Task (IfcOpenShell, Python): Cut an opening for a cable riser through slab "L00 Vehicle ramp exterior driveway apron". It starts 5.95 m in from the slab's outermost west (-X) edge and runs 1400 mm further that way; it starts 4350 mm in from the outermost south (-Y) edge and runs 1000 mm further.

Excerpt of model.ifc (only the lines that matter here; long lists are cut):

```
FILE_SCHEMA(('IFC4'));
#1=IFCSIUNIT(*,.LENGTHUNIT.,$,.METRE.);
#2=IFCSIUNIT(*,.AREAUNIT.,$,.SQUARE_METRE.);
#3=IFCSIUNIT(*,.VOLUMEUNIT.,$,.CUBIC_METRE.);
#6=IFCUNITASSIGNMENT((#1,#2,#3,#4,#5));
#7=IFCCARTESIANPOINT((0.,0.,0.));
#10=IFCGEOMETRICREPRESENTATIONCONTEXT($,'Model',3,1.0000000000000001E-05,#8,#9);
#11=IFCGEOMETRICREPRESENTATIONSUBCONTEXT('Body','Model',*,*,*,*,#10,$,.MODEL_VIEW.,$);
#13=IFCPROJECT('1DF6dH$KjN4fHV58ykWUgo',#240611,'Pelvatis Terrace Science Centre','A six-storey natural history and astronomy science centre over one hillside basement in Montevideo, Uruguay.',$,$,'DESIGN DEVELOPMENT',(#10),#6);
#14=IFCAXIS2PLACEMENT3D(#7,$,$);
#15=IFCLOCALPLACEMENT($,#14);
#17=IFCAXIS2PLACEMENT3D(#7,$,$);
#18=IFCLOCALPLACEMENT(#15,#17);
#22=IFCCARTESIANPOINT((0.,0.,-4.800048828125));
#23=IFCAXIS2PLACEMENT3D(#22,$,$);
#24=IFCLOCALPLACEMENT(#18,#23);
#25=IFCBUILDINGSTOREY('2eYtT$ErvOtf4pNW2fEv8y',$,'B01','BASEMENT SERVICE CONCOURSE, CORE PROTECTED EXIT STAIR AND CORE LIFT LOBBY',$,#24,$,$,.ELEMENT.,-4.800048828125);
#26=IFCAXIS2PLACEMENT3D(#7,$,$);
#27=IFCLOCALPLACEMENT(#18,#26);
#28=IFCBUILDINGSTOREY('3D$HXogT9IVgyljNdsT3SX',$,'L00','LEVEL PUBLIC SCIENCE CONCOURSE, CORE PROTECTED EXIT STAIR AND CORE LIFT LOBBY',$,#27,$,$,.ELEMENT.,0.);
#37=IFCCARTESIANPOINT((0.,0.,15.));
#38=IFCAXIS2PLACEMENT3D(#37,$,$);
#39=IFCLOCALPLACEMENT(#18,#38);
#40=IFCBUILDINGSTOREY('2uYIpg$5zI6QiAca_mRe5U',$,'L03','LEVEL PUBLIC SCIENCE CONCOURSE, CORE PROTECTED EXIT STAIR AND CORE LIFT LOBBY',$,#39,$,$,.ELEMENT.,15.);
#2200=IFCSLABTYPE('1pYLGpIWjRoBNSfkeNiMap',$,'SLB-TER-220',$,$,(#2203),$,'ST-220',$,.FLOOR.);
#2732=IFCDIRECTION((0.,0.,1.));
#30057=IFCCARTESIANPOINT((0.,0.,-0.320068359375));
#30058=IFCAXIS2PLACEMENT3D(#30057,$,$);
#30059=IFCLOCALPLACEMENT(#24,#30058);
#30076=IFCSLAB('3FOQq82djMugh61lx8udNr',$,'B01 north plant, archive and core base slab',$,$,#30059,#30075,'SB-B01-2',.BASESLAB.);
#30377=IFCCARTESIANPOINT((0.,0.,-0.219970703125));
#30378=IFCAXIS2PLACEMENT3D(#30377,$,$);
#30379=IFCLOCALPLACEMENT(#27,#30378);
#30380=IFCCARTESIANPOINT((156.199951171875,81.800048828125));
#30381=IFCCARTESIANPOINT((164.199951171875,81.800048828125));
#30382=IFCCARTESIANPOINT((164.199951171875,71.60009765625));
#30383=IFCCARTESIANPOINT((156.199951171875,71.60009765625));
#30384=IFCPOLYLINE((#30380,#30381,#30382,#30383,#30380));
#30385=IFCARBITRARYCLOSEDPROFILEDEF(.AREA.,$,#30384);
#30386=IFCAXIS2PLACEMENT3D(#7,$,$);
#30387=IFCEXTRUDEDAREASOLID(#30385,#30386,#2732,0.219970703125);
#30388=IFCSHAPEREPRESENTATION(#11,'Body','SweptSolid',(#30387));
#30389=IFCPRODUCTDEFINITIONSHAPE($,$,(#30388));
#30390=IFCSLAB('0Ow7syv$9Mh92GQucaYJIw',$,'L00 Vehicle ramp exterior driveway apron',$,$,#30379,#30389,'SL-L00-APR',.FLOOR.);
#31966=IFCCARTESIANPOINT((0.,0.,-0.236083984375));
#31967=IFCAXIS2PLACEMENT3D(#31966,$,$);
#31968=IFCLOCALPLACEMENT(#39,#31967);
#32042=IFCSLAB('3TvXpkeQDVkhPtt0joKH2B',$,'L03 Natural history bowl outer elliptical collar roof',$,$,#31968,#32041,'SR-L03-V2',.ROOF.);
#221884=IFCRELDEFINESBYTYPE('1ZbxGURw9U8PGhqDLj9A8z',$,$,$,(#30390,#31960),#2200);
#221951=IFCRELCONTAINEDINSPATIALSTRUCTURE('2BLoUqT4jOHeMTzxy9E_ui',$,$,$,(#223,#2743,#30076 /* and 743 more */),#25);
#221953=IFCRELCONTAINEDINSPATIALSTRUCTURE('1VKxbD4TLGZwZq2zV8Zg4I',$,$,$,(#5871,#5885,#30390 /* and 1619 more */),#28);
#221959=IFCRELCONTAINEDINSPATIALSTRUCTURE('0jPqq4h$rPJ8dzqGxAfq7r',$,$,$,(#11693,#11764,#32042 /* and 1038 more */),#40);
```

```python
import numpy as np
import ifcopenshell
import ifcopenshell.api.feature
import ifcopenshell.api.geometry
import ifcopenshell.api.root
import ifcopenshell.geom
import ifcopenshell.util.placement
import ifcopenshell.util.representation
import ifcopenshell.util.shape
import ifcopenshell.util.unit

model = ifcopenshell.open("model.ifc")
unit_scale = ifcopenshell.util.unit.calculate_unit_scale(model)
settings = ifcopenshell.geom.settings()


def volume(element):
    """Net volume in cubic metres, openings subtracted."""
    shape = ifcopenshell.geom.create_shape(settings, element)
    return ifcopenshell.util.shape.get_volume(shape.geometry)


slab = model.by_guid("0Ow7syv$9Mh92GQucaYJIw")
before = volume(slab)

# Extent in the slab's own axes, in metres. The edges named are its -X and -Y sides.
slab_shape = ifcopenshell.geom.create_shape(settings, slab)
vertices = ifcopenshell.util.shape.get_vertices(slab_shape.geometry)
x_min, y_min, bottom = vertices.min(axis=0)
top = vertices[:, 2].max()

opening = ifcopenshell.api.root.create_entity(model, ifc_class="IfcOpeningElement", name="Cable riser opening", predefined_type="OPENING")
context = ifcopenshell.util.representation.get_context(model, "Model", "Body", "MODEL_VIEW")
width, depth = 1.4, 1
outline = [(0.0, 0.0), (width, 0.0), (width, depth), (0.0, depth), (0.0, 0.0)]
# Overshoot both faces by 50 mm so the cut is clean.
shape = ifcopenshell.api.geometry.add_slab_representation(
    model, context=context, depth=top - bottom + 0.1, polyline=outline
)
ifcopenshell.api.geometry.assign_representation(model, product=opening, representation=shape)

matrix = ifcopenshell.util.placement.get_local_placement(slab.ObjectPlacement)
matrix[:, 3] = matrix @ np.append(np.array([x_min + 5.95, y_min + 4.35, bottom - 0.05]) / unit_scale, 1.0)
ifcopenshell.api.geometry.edit_object_placement(model, product=opening, matrix=matrix, is_si=False)
ifcopenshell.api.feature.add_feature(model, feature=opening, element=slab)

after = volume(slab)

print(f"slab volume {before:.3f} -> {after:.3f} m3")

model.write("model_v2.ifc")
```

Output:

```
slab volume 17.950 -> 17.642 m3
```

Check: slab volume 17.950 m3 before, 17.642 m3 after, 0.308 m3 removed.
